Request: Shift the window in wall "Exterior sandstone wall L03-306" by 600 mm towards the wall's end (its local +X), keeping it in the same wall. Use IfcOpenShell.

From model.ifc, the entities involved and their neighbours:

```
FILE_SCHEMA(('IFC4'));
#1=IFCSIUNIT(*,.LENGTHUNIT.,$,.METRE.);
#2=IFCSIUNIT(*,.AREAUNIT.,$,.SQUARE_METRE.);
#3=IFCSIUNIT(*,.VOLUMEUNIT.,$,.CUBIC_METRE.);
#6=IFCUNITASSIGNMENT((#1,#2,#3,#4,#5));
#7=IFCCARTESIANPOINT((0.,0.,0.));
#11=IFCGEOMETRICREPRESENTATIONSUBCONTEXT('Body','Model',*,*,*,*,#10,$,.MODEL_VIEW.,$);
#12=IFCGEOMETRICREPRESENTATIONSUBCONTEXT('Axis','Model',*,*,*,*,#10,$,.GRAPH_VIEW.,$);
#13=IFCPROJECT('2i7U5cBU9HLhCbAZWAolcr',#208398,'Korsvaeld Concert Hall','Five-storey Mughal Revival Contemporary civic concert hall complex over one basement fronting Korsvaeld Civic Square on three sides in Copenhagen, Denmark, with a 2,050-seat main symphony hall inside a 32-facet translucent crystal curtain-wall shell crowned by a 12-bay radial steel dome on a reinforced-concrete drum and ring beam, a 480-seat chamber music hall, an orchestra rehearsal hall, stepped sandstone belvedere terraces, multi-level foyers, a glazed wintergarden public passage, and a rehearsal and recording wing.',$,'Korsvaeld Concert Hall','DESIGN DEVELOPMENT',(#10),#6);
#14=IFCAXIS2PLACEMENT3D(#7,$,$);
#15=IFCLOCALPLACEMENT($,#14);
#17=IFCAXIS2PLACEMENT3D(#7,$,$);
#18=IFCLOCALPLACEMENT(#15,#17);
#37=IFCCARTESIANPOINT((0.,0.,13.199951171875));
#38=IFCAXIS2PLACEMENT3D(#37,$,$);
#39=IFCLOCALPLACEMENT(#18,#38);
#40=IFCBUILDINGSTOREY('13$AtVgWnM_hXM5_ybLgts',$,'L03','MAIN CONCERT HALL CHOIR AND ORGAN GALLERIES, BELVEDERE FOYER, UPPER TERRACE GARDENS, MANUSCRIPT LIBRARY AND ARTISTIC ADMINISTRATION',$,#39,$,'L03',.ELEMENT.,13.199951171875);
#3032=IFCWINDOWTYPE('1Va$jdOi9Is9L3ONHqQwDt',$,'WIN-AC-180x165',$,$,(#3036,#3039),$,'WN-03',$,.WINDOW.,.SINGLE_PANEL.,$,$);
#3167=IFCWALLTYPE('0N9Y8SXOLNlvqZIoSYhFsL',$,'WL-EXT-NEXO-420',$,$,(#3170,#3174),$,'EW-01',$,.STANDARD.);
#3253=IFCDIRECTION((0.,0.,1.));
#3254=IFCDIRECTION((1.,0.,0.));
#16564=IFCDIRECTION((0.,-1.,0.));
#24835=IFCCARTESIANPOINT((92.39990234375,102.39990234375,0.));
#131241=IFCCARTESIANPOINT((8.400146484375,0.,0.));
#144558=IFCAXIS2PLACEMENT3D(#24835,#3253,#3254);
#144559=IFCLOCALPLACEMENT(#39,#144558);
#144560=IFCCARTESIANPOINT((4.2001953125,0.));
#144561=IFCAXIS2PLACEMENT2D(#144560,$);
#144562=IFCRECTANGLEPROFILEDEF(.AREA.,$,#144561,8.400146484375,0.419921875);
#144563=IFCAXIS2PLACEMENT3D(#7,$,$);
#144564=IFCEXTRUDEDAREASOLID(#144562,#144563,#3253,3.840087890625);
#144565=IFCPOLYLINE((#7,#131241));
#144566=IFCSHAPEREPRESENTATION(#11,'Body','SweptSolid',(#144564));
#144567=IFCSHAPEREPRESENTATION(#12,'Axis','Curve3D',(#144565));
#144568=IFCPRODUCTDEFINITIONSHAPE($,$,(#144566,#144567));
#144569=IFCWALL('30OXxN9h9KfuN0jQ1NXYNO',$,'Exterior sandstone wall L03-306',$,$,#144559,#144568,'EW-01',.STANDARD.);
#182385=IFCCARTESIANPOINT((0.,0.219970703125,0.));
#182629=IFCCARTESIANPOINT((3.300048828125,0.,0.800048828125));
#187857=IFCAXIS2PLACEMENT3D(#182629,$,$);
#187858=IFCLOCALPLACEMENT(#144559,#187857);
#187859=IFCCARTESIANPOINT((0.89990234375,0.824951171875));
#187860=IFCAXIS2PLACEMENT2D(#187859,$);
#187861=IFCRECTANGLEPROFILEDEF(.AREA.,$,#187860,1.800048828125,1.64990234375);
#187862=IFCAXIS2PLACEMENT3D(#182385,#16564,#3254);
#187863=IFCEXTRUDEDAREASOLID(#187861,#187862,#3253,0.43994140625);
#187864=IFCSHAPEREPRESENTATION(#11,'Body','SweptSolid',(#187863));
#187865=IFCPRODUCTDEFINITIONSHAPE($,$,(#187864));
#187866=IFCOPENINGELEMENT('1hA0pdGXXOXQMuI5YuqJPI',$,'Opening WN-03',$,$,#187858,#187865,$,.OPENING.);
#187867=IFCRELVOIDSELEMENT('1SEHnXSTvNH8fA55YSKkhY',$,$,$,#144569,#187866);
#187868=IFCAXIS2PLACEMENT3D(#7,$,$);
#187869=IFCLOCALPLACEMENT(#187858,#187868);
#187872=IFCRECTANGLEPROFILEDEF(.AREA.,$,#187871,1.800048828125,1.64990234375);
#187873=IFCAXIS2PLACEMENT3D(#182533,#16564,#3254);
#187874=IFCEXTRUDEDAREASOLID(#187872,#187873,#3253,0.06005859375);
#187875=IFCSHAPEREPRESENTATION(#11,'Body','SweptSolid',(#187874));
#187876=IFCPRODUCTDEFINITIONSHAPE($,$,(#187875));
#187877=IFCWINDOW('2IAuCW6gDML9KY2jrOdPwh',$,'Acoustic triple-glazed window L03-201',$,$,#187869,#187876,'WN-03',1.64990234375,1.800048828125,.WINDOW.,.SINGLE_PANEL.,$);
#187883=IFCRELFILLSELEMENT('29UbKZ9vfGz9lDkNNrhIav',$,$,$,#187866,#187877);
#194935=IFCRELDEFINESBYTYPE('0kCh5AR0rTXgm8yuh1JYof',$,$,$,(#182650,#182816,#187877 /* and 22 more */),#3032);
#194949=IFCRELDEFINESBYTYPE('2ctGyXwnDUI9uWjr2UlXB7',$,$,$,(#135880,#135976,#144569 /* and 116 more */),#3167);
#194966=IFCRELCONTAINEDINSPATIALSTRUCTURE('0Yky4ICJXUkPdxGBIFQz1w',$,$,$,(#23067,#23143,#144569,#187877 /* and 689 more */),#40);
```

```python
import ifcopenshell
import ifcopenshell.api.geometry
import ifcopenshell.util.placement
import ifcopenshell.util.unit

model = ifcopenshell.open("model.ifc")
unit_scale = ifcopenshell.util.unit.calculate_unit_scale(model)

window = model.by_guid("2IAuCW6gDML9KY2jrOdPwh")
opening = window.FillsVoids[0].RelatingOpeningElement
wall = opening.VoidsElements[0].RelatingBuildingElement

wall_matrix = ifcopenshell.util.placement.get_local_placement(wall.ObjectPlacement)
shift = wall_matrix[:3, 0] * 0.6 / unit_scale
before = ifcopenshell.util.placement.get_local_placement(window.ObjectPlacement)[:3, 3].copy()

# The window is placed relative to its opening, so it follows when the opening moves.
matrix = ifcopenshell.util.placement.get_local_placement(opening.ObjectPlacement)
matrix[:3, 3] += shift
ifcopenshell.api.geometry.edit_object_placement(
    model, product=opening, matrix=matrix, is_si=False, should_transform_children=True
)

after = ifcopenshell.util.placement.get_local_placement(window.ObjectPlacement)[:3, 3]
print("window moved by", (after - before).round(3) + 0.0)

model.write("model_v2.ifc")
```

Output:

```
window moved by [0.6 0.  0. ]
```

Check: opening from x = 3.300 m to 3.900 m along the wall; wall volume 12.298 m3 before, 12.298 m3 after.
